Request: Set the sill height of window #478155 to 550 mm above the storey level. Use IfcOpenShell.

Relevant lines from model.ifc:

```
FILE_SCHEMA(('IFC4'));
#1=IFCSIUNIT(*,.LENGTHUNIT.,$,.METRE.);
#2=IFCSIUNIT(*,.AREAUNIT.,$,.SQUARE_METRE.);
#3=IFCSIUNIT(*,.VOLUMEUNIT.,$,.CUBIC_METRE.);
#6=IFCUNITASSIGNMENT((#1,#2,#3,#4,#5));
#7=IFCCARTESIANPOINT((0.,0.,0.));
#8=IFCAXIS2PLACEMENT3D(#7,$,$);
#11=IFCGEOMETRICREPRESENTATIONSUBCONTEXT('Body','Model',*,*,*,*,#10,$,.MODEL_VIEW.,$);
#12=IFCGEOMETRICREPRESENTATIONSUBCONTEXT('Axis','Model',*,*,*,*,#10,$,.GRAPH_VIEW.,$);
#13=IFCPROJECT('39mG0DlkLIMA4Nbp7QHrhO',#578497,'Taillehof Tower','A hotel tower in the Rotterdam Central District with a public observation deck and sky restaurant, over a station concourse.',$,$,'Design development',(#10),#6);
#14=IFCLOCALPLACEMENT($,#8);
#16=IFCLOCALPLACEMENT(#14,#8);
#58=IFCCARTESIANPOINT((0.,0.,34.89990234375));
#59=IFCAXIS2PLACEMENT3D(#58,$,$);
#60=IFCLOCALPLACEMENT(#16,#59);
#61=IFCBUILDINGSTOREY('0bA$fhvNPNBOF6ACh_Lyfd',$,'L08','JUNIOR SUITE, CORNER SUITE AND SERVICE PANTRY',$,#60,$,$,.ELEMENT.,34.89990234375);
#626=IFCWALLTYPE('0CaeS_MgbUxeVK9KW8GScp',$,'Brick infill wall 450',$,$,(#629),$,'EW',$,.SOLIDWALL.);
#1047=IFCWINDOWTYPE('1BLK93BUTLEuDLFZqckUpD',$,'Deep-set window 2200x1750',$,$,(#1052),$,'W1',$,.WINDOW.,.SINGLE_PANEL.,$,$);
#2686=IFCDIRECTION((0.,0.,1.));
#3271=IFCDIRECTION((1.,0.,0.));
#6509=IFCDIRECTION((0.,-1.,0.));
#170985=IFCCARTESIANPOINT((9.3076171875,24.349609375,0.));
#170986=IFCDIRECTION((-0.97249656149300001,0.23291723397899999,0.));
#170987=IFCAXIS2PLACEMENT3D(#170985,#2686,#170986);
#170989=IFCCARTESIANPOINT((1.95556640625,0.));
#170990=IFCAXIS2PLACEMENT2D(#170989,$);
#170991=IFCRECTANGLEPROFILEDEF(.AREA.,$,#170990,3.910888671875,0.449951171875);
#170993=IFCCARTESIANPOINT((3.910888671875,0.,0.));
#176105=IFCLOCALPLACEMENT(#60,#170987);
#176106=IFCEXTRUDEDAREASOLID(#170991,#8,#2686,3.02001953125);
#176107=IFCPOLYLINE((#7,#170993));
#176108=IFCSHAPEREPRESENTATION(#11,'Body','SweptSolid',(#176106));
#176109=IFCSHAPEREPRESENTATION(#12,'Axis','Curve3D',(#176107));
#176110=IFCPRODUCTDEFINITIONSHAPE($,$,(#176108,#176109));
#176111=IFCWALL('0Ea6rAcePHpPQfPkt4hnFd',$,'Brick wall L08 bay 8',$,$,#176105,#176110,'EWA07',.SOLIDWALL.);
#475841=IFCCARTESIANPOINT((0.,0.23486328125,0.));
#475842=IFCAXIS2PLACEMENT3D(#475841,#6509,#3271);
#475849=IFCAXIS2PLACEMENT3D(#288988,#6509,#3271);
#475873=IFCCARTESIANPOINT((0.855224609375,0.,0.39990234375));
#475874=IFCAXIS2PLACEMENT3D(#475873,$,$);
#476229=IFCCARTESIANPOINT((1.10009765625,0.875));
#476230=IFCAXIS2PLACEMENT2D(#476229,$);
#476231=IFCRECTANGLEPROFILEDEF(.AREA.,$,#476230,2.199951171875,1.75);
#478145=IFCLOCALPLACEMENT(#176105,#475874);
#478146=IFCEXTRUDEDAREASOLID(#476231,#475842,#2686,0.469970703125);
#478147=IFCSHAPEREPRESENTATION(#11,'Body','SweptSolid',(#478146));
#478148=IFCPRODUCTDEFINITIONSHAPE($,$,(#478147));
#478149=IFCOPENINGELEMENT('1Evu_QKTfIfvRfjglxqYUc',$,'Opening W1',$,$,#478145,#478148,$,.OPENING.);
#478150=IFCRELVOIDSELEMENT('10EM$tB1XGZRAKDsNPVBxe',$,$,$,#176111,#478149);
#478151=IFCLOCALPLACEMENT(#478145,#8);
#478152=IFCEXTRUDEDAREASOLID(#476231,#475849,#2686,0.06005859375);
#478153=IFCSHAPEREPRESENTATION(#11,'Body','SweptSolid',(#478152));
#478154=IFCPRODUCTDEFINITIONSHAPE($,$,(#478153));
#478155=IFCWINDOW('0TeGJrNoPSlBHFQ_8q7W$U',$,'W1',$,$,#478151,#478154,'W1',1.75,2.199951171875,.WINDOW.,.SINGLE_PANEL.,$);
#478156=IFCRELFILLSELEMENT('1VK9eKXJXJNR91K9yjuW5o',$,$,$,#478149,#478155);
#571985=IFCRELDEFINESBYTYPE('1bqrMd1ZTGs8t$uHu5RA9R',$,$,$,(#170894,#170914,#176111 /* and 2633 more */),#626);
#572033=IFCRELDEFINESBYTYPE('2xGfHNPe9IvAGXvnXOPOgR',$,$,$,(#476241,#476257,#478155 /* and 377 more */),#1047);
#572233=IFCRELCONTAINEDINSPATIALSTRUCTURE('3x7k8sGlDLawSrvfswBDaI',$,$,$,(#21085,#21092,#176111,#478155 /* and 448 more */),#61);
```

```python
import numpy as np
import ifcopenshell
import ifcopenshell.api.geometry
import ifcopenshell.geom
import ifcopenshell.util.element
import ifcopenshell.util.placement
import ifcopenshell.util.shape
import ifcopenshell.util.unit

model = ifcopenshell.open("model.ifc")
unit_scale = ifcopenshell.util.unit.calculate_unit_scale(model)

window = model.by_id(478155)
opening = window.FillsVoids[0].RelatingOpeningElement
storey = ifcopenshell.util.element.get_container(window, ifc_class="IfcBuildingStorey")
level = ifcopenshell.util.placement.get_local_placement(storey.ObjectPlacement)[2, 3]

# The opening's origin need not be at the sill, so measure its lowest point.
shape = ifcopenshell.geom.create_shape(ifcopenshell.geom.settings(), opening)
bottom = ifcopenshell.util.shape.get_shape_bottom_elevation(shape, shape.geometry) / unit_scale
dz = level + 0.55 / unit_scale - bottom

shift = np.array([0.0, 0.0, dz])
# The window is placed relative to its opening, so it follows when the opening moves.
matrix = ifcopenshell.util.placement.get_local_placement(opening.ObjectPlacement)
matrix[:3, 3] += shift
ifcopenshell.api.geometry.edit_object_placement(
    model, product=opening, matrix=matrix, is_si=False, should_transform_children=True
)

print(f"moved by {dz * unit_scale:+.3f} m")

model.write("model_edited.ifc")
```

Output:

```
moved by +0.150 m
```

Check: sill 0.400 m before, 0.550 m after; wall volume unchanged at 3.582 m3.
